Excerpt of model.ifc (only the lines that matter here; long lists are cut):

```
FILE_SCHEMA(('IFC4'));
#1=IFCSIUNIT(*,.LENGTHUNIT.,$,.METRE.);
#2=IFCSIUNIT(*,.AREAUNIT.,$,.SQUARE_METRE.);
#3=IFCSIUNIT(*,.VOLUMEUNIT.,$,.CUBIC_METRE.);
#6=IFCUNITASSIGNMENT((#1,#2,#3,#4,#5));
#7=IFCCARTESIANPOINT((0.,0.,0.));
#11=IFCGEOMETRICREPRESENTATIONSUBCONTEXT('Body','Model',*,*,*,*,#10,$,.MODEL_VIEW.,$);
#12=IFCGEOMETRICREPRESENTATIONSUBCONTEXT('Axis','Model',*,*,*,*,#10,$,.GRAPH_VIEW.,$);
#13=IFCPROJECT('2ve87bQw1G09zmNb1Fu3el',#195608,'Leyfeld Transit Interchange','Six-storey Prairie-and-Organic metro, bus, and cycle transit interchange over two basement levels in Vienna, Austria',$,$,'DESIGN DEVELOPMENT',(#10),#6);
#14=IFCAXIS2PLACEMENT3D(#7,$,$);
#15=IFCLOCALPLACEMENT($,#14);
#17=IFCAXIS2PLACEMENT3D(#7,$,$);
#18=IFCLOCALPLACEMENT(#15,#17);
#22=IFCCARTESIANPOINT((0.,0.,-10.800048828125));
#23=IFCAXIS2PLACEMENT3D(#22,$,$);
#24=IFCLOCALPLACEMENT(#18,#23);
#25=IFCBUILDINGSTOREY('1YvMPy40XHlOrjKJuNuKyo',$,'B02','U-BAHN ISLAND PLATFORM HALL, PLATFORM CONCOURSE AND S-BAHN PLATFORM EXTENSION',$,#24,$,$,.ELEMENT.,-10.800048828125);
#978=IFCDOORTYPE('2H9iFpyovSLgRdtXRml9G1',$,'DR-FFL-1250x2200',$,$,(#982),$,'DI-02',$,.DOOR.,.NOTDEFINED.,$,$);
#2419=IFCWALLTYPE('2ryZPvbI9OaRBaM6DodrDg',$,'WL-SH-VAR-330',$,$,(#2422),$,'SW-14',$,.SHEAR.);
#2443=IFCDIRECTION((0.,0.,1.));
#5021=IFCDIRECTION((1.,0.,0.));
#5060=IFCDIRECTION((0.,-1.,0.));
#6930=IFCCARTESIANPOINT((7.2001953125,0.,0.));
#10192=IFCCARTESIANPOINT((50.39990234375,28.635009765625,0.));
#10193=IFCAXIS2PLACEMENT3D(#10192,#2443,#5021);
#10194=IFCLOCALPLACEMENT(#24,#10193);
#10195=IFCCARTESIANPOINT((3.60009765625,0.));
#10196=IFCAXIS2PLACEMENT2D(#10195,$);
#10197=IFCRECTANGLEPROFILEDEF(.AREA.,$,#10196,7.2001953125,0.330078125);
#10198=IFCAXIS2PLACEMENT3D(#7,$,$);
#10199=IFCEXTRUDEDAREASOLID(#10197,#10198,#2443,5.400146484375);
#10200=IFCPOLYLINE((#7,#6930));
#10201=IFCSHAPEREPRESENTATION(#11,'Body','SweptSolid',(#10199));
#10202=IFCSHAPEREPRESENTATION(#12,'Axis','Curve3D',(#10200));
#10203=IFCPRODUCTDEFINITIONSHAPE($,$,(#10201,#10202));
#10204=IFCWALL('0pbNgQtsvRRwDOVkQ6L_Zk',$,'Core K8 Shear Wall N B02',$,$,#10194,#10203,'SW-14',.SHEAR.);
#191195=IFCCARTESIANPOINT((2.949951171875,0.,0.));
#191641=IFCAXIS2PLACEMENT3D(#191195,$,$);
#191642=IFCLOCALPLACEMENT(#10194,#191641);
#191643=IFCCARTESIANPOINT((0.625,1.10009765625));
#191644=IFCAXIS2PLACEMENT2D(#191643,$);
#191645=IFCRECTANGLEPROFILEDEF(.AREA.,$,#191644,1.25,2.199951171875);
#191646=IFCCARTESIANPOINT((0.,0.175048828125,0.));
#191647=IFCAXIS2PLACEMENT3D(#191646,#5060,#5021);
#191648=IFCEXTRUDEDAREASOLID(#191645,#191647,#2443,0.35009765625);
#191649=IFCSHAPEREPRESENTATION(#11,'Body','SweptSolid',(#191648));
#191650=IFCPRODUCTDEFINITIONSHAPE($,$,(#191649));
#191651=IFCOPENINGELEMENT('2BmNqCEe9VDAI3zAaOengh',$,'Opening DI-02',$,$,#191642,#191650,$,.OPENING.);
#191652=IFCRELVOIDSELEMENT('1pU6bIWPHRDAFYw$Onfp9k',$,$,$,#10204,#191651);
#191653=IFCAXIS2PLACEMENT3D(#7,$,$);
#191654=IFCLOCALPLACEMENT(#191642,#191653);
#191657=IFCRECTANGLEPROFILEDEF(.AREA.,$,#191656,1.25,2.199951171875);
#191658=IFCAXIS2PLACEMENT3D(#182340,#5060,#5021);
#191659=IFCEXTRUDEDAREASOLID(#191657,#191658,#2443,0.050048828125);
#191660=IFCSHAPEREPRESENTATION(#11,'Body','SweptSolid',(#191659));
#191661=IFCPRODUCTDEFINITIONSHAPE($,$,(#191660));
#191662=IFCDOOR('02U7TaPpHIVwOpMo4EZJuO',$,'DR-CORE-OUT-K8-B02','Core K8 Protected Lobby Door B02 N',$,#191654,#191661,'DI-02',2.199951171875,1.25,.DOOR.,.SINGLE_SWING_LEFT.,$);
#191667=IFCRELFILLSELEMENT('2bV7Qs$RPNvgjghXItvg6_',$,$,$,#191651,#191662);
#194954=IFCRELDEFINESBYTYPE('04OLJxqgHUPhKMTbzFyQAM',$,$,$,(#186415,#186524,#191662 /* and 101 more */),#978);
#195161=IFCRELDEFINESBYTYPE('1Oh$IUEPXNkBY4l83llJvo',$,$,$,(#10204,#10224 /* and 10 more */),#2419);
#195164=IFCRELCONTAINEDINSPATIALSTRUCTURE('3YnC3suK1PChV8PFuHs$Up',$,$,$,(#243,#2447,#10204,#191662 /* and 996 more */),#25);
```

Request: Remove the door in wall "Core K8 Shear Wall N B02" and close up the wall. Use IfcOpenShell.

```python
import ifcopenshell
import ifcopenshell.api.feature
import ifcopenshell.api.root
import ifcopenshell.geom
import ifcopenshell.util.shape

model = ifcopenshell.open("model.ifc")
settings = ifcopenshell.geom.settings()


def volume(element):
    """Net volume in cubic metres, openings subtracted."""
    shape = ifcopenshell.geom.create_shape(settings, element)
    return ifcopenshell.util.shape.get_volume(shape.geometry)


door = model.by_id(191662)
opening = door.FillsVoids[0].RelatingOpeningElement
wall = opening.VoidsElements[0].RelatingBuildingElement
before = volume(wall)

ifcopenshell.api.root.remove_product(model, product=door)
ifcopenshell.api.feature.remove_feature(model, feature=opening)

after = volume(wall)

print(f"wall volume {before:.3f} -> {after:.3f} m3")

model.write("model_updated.ifc")
```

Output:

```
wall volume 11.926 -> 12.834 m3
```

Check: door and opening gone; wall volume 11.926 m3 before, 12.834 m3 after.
